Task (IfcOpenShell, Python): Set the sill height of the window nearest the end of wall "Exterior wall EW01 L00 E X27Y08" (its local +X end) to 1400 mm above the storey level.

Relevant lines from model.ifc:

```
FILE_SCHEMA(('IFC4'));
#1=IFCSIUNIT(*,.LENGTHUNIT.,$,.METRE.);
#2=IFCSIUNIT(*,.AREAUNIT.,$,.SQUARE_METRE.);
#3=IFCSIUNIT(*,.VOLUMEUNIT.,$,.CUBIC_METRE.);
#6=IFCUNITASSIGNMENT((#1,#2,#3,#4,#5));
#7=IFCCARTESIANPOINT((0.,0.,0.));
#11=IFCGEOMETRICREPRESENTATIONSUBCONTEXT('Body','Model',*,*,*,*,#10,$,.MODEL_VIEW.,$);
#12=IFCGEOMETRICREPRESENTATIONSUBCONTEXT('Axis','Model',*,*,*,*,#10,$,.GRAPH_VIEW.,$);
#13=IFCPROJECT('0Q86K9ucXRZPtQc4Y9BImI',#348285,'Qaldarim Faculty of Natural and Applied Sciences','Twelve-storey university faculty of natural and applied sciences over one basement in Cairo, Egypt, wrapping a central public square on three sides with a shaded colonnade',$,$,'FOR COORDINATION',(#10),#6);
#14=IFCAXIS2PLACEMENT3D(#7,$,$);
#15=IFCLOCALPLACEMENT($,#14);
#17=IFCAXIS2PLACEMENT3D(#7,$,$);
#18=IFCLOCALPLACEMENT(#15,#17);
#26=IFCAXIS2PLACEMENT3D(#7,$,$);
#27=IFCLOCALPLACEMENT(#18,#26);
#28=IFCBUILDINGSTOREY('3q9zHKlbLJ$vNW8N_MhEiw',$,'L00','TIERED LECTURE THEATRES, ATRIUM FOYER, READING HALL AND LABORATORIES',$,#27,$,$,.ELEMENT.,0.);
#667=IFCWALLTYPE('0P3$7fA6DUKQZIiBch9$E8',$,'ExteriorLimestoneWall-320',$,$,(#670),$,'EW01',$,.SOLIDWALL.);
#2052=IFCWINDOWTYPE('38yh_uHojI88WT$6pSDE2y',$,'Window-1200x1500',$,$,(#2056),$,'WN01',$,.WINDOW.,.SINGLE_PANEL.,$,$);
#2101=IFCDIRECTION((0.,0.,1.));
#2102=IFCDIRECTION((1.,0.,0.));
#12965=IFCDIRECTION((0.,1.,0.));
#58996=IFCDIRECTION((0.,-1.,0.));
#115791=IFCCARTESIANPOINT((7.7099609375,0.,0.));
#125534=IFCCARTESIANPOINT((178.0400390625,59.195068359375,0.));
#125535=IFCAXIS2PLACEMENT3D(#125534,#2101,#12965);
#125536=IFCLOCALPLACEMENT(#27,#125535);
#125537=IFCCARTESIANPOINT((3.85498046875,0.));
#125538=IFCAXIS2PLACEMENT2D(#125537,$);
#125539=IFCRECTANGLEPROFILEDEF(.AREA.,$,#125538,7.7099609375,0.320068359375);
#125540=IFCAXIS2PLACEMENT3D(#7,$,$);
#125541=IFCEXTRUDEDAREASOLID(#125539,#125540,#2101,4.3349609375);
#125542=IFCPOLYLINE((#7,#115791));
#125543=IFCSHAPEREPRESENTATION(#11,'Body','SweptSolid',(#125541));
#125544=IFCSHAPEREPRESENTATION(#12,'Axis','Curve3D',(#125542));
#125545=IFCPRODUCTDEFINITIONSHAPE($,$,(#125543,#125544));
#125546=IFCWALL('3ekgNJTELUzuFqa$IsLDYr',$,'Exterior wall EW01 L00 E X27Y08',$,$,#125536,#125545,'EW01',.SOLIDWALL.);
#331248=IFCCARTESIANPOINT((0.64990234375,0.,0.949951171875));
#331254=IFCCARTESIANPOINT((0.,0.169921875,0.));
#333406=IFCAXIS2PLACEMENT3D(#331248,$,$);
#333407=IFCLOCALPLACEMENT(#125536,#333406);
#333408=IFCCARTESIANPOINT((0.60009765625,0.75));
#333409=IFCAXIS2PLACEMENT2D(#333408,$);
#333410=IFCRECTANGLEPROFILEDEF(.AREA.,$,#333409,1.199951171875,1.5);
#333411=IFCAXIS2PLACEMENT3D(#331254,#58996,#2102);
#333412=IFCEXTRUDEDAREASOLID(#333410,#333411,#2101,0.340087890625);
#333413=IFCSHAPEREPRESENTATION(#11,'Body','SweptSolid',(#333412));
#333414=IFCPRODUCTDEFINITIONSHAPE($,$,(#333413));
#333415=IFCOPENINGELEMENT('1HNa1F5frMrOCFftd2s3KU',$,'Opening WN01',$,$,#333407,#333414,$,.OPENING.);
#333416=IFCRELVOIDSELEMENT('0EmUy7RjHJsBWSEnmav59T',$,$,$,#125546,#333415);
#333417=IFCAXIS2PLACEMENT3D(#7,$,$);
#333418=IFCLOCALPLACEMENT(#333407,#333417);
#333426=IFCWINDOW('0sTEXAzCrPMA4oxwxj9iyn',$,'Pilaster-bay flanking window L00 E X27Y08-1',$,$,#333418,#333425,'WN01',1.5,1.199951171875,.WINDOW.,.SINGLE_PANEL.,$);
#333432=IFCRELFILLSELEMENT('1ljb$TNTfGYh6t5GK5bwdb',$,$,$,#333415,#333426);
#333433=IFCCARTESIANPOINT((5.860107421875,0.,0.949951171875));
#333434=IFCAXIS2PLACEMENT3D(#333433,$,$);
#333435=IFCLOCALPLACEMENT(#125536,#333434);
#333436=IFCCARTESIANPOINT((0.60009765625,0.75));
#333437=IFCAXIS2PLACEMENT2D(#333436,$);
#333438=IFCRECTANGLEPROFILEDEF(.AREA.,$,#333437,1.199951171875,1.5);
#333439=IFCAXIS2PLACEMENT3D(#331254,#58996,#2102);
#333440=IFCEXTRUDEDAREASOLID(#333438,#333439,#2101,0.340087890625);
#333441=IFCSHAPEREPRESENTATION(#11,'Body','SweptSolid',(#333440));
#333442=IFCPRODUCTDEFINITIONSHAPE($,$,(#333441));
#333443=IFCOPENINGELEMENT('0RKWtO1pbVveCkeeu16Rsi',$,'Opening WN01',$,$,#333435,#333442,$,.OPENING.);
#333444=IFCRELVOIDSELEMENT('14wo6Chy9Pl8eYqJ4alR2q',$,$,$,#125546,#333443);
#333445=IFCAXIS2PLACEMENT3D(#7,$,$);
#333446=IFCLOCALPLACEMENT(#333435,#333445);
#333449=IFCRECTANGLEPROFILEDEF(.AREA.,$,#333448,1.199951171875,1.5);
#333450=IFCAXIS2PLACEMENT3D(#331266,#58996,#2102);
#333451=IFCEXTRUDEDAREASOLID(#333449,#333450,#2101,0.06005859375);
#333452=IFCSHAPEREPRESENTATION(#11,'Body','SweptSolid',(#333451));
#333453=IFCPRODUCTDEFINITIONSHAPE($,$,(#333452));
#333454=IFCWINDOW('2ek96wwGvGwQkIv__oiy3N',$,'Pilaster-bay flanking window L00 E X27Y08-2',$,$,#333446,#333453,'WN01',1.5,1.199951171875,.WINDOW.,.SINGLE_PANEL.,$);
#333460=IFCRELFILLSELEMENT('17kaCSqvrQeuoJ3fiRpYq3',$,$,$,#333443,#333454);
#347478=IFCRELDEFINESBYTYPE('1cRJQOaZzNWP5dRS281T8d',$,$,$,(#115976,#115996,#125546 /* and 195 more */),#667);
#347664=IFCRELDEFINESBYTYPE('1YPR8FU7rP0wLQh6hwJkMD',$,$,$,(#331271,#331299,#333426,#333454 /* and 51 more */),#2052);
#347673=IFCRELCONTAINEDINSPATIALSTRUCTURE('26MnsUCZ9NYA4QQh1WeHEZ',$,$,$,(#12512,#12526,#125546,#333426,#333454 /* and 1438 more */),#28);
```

```python
import numpy as np
import ifcopenshell
import ifcopenshell.api.geometry
import ifcopenshell.geom
import ifcopenshell.util.element
import ifcopenshell.util.placement
import ifcopenshell.util.shape
import ifcopenshell.util.unit

model = ifcopenshell.open("model.ifc")
unit_scale = ifcopenshell.util.unit.calculate_unit_scale(model)

window = model.by_guid("2ek96wwGvGwQkIv__oiy3N")
opening = window.FillsVoids[0].RelatingOpeningElement
storey = ifcopenshell.util.element.get_container(window, ifc_class="IfcBuildingStorey")
level = ifcopenshell.util.placement.get_local_placement(storey.ObjectPlacement)[2, 3]

# The opening's origin need not be at the sill, so measure its lowest point.
shape = ifcopenshell.geom.create_shape(ifcopenshell.geom.settings(), opening)
bottom = ifcopenshell.util.shape.get_shape_bottom_elevation(shape, shape.geometry) / unit_scale
dz = level + 1.4 - bottom

shift = np.array([0.0, 0.0, dz])
# The window is placed relative to its opening, so it follows when the opening moves.
matrix = ifcopenshell.util.placement.get_local_placement(opening.ObjectPlacement)
matrix[:3, 3] += shift
ifcopenshell.api.geometry.edit_object_placement(
    model, product=opening, matrix=matrix, is_si=False, should_transform_children=True
)

print(f"moved by {dz * unit_scale:+.3f} m")

model.write("model_rev.ifc")
```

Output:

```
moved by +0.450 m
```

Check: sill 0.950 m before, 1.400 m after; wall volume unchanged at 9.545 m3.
